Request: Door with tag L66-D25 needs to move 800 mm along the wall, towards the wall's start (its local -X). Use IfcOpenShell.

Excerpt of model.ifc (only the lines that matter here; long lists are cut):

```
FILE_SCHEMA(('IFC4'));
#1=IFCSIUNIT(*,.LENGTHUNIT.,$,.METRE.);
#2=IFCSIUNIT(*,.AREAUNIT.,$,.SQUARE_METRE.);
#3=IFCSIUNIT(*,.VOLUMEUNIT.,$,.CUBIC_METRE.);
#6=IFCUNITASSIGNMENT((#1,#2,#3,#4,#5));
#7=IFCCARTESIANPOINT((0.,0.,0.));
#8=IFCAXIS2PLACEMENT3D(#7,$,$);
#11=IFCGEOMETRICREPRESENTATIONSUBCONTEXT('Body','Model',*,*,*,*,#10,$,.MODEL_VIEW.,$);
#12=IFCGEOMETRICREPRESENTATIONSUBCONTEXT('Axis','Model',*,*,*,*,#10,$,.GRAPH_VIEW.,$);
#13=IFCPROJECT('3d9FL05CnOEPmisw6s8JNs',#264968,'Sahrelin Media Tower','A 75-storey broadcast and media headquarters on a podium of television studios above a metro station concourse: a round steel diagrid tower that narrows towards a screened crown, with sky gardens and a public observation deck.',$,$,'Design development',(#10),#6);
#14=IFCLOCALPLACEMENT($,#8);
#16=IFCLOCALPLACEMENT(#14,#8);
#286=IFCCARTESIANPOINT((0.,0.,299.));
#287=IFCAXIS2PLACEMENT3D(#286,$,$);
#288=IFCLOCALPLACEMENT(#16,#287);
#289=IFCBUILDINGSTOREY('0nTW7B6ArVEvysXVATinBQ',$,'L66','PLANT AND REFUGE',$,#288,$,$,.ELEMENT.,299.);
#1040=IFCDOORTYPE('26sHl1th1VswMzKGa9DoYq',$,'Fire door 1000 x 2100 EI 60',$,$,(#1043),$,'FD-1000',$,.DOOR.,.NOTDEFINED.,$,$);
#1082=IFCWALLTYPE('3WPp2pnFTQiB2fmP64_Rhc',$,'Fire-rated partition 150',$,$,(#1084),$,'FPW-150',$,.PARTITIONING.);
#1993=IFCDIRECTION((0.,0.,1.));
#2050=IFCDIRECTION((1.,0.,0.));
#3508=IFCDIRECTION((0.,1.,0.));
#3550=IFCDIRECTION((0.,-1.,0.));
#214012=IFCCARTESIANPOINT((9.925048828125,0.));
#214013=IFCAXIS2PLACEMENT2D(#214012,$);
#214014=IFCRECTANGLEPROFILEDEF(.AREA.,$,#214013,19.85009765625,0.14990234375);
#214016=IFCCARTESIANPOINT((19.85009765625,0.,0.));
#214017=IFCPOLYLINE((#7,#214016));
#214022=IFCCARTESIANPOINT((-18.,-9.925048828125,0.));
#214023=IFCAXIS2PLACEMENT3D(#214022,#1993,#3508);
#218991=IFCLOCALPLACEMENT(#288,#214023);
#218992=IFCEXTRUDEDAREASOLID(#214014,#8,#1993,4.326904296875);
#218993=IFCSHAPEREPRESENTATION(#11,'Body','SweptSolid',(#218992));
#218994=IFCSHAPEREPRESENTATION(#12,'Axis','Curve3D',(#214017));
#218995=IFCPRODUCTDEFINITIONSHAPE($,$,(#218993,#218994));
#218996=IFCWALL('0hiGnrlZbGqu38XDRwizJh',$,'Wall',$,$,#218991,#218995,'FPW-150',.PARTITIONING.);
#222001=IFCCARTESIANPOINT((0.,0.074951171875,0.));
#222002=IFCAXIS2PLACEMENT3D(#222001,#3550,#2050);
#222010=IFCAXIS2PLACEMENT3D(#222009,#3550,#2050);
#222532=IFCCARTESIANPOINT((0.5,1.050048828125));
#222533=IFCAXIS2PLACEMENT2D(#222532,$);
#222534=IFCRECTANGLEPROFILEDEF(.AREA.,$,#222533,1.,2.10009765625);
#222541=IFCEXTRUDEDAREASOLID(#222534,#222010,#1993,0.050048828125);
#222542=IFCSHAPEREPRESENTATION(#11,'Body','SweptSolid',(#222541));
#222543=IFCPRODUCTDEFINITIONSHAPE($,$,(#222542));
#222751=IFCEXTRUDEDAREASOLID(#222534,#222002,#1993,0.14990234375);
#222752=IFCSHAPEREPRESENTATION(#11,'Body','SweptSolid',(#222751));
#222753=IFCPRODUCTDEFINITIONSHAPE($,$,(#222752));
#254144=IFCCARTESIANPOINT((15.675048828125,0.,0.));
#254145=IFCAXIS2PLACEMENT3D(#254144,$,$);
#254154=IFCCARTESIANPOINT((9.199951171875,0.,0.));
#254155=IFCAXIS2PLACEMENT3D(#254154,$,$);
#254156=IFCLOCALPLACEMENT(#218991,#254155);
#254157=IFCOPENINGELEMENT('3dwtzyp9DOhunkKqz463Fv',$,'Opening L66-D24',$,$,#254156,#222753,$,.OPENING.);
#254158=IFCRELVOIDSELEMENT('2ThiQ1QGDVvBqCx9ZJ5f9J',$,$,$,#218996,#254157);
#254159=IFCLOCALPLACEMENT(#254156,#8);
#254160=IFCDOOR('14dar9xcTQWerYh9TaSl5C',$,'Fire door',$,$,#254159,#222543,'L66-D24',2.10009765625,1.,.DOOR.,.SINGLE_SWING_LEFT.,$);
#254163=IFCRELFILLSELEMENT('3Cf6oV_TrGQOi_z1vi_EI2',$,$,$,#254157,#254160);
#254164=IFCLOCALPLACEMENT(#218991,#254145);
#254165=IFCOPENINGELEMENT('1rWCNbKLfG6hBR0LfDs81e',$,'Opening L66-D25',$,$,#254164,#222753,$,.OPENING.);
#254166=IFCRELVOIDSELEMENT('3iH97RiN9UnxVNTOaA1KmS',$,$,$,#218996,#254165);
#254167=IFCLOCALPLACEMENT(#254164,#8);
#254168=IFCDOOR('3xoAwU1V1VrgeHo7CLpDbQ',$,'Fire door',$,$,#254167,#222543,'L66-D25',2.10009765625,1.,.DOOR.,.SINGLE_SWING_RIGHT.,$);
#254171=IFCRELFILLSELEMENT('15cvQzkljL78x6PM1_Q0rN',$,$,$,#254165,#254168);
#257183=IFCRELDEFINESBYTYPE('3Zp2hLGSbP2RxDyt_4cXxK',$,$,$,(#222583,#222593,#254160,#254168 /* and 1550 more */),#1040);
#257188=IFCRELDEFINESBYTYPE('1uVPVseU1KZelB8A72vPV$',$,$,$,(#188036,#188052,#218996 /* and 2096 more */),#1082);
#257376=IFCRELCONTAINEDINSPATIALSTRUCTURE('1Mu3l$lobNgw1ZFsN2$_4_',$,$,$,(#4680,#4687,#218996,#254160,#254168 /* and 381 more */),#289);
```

```python
import ifcopenshell
import ifcopenshell.api.geometry
import ifcopenshell.util.placement

model = ifcopenshell.open("model.ifc")

door = model.by_guid("3xoAwU1V1VrgeHo7CLpDbQ")
opening = door.FillsVoids[0].RelatingOpeningElement
wall = opening.VoidsElements[0].RelatingBuildingElement

wall_matrix = ifcopenshell.util.placement.get_local_placement(wall.ObjectPlacement)
shift = wall_matrix[:3, 0] * -0.8
before = ifcopenshell.util.placement.get_local_placement(door.ObjectPlacement)[:3, 3].copy()

# The door is placed relative to its opening, so it follows when the opening moves.
matrix = ifcopenshell.util.placement.get_local_placement(opening.ObjectPlacement)
matrix[:3, 3] += shift
ifcopenshell.api.geometry.edit_object_placement(
    model, product=opening, matrix=matrix, is_si=False, should_transform_children=True
)

after = ifcopenshell.util.placement.get_local_placement(door.ObjectPlacement)[:3, 3]
print("door moved by", (after - before).round(3) + 0.0)

model.write("model_v2.ifc")
```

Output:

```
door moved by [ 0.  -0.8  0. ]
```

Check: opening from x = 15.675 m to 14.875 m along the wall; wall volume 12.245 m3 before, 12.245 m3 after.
